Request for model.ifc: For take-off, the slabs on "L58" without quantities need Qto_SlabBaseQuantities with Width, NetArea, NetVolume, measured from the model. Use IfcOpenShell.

First a look at what the model holds.

```python
import ifcopenshell
import ifcopenshell.util.element
import ifcopenshell.util.unit

model = ifcopenshell.open("model.ifc")
print(model.schema)
for unit_type in ("LENGTHUNIT", "AREAUNIT", "VOLUMEUNIT"):
    print(unit_type, ifcopenshell.util.unit.calculate_unit_scale(model, unit_type))
storey = next(s for s in model.by_type("IfcBuildingStorey") if s.Name == "L58")
slabs = [e for e in ifcopenshell.util.element.get_decomposition(storey) if e.is_a("IfcSlab")]
for e in sorted(slabs, key=lambda e: e.id()):
    print(e.id(), e.is_a(), e.Name, list(ifcopenshell.util.element.get_psets(e, qtos_only=True)), sep=" | ")
```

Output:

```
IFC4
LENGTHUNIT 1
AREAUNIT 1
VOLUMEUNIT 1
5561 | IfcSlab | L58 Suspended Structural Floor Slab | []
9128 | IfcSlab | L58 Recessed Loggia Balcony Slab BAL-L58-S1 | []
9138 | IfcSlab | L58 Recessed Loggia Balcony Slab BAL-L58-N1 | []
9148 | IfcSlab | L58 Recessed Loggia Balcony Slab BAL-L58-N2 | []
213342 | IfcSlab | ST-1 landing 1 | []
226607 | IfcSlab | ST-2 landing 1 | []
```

```python
import ifcopenshell
import ifcopenshell.api.pset
import ifcopenshell.geom
import ifcopenshell.util.element
import ifcopenshell.util.shape
import ifcopenshell.util.unit

model = ifcopenshell.open("model.ifc")
unit_scale = ifcopenshell.util.unit.calculate_unit_scale(model)
area_scale = ifcopenshell.util.unit.calculate_unit_scale(model, "AREAUNIT")
volume_scale = ifcopenshell.util.unit.calculate_unit_scale(model, "VOLUMEUNIT")
settings = ifcopenshell.geom.settings()

storey = next(s for s in model.by_type("IfcBuildingStorey") if s.Name == "L58")
slabs = [e for e in ifcopenshell.util.element.get_decomposition(storey) if e.is_a("IfcSlab")]

for e in sorted(slabs, key=lambda e: e.id()):
    if ifcopenshell.util.element.get_psets(e, qtos_only=True, should_inherit=False):
        continue
    # Geometry comes back in metres, in the element's own axes.
    shape = ifcopenshell.geom.create_shape(settings, e)
    values = {
        "Width": ifcopenshell.util.shape.get_z(shape.geometry) / unit_scale,
        "NetArea": ifcopenshell.util.shape.get_footprint_area(shape.geometry) / area_scale,
        "NetVolume": ifcopenshell.util.shape.get_volume(shape.geometry) / volume_scale,
    }
    qto = ifcopenshell.api.pset.add_qto(model, product=e, name="Qto_SlabBaseQuantities")
    ifcopenshell.api.pset.edit_qto(model, qto=qto, properties=values)
    print(e.id(), {k: round(v, 3) for k, v in values.items()})

model.write("model_edited.ifc")
```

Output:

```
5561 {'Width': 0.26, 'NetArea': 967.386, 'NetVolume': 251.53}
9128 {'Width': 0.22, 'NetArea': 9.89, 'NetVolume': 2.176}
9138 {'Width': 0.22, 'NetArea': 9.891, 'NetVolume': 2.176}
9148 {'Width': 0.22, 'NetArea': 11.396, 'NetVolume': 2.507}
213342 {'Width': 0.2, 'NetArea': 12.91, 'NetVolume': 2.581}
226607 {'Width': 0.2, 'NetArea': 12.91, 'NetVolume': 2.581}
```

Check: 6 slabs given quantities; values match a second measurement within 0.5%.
